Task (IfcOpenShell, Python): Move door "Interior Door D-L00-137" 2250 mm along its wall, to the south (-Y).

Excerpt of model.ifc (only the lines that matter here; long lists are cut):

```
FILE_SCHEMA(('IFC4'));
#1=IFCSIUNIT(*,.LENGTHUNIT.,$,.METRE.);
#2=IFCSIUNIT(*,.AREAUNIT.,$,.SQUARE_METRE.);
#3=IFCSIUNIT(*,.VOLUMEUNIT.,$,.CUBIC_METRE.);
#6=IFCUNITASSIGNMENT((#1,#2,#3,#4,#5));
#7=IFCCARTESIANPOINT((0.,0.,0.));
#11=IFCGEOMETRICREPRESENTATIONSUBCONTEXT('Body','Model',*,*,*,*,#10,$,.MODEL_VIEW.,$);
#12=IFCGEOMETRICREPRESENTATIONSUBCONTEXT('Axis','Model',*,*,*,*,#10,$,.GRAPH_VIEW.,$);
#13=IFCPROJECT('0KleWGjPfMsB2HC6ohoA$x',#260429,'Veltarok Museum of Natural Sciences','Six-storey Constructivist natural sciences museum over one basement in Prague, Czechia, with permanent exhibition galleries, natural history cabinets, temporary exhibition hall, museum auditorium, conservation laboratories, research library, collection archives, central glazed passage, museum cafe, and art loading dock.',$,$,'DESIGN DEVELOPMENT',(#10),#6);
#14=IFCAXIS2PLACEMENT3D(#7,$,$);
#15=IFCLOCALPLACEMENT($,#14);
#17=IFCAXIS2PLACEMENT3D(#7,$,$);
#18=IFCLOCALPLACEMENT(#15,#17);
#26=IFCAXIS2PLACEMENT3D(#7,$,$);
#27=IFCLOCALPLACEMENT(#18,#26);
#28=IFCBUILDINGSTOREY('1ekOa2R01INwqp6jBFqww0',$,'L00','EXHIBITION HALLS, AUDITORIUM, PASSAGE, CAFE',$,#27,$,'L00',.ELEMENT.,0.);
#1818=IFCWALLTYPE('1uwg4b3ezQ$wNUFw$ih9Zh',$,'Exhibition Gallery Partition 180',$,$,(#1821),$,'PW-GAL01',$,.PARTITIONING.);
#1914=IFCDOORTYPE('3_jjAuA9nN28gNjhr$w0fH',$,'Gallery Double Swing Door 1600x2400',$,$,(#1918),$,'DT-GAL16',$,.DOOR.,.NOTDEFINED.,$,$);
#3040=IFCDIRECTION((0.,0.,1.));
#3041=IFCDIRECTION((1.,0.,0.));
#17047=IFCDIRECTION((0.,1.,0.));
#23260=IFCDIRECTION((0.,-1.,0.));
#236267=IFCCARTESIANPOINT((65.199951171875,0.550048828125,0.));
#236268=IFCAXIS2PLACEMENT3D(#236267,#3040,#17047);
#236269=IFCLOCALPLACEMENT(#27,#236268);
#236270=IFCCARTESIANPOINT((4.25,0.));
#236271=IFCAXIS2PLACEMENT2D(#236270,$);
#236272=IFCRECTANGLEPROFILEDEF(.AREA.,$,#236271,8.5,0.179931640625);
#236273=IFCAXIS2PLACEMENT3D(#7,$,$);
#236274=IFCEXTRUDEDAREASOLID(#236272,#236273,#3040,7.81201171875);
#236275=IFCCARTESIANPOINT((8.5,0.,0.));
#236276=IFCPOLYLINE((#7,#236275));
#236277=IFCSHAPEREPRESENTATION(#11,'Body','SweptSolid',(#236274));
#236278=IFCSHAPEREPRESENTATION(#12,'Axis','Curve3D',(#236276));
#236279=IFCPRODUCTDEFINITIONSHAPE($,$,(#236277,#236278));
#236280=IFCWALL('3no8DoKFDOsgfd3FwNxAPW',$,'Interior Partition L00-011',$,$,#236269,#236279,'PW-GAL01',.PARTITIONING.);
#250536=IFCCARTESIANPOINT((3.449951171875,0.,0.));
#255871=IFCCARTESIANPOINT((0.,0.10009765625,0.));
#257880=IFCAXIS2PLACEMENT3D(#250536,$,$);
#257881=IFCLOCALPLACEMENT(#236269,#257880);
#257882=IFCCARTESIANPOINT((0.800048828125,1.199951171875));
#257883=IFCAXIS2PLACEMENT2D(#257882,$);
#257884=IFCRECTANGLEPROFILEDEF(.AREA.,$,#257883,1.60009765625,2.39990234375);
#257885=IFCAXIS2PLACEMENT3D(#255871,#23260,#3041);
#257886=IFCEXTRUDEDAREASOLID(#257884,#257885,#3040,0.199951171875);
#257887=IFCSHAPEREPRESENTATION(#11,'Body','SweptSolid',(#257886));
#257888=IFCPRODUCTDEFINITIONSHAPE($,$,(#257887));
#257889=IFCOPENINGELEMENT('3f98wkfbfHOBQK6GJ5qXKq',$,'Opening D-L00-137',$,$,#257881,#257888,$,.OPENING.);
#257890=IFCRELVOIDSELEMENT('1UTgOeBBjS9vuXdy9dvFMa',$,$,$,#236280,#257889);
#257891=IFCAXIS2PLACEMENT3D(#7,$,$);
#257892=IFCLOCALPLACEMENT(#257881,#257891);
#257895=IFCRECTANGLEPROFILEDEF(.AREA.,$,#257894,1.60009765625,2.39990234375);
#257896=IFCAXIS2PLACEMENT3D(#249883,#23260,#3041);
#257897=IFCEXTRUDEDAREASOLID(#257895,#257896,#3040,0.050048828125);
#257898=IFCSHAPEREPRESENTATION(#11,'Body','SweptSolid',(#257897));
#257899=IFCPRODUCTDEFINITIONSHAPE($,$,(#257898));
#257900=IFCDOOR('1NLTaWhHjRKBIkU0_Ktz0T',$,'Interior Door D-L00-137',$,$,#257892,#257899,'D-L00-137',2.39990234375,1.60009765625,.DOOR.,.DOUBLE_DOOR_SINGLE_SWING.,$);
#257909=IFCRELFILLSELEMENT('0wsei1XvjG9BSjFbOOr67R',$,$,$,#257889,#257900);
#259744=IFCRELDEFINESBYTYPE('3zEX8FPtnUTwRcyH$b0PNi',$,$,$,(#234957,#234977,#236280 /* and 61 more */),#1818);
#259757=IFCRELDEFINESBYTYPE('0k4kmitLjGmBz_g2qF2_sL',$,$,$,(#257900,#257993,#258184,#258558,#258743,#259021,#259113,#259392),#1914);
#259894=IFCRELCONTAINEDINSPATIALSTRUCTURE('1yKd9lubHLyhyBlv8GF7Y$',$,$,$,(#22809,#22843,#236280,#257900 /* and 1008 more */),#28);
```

```python
import ifcopenshell
import ifcopenshell.api.geometry
import ifcopenshell.util.placement
import ifcopenshell.util.unit

model = ifcopenshell.open("model.ifc")
unit_scale = ifcopenshell.util.unit.calculate_unit_scale(model)

door = model.by_guid("1NLTaWhHjRKBIkU0_Ktz0T")
opening = door.FillsVoids[0].RelatingOpeningElement
wall = opening.VoidsElements[0].RelatingBuildingElement

wall_matrix = ifcopenshell.util.placement.get_local_placement(wall.ObjectPlacement)
shift = wall_matrix[:3, 0] * -2.25 / unit_scale
before = ifcopenshell.util.placement.get_local_placement(door.ObjectPlacement)[:3, 3].copy()

# The door is placed relative to its opening, so it follows when the opening moves.
matrix = ifcopenshell.util.placement.get_local_placement(opening.ObjectPlacement)
matrix[:3, 3] += shift
ifcopenshell.api.geometry.edit_object_placement(
    model, product=opening, matrix=matrix, is_si=False, should_transform_children=True
)

after = ifcopenshell.util.placement.get_local_placement(door.ObjectPlacement)[:3, 3]
print("door moved by", (after - before).round(3) + 0.0)

model.write("model-out.ifc")
```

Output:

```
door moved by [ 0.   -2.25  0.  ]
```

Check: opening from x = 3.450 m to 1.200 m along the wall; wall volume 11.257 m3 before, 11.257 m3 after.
